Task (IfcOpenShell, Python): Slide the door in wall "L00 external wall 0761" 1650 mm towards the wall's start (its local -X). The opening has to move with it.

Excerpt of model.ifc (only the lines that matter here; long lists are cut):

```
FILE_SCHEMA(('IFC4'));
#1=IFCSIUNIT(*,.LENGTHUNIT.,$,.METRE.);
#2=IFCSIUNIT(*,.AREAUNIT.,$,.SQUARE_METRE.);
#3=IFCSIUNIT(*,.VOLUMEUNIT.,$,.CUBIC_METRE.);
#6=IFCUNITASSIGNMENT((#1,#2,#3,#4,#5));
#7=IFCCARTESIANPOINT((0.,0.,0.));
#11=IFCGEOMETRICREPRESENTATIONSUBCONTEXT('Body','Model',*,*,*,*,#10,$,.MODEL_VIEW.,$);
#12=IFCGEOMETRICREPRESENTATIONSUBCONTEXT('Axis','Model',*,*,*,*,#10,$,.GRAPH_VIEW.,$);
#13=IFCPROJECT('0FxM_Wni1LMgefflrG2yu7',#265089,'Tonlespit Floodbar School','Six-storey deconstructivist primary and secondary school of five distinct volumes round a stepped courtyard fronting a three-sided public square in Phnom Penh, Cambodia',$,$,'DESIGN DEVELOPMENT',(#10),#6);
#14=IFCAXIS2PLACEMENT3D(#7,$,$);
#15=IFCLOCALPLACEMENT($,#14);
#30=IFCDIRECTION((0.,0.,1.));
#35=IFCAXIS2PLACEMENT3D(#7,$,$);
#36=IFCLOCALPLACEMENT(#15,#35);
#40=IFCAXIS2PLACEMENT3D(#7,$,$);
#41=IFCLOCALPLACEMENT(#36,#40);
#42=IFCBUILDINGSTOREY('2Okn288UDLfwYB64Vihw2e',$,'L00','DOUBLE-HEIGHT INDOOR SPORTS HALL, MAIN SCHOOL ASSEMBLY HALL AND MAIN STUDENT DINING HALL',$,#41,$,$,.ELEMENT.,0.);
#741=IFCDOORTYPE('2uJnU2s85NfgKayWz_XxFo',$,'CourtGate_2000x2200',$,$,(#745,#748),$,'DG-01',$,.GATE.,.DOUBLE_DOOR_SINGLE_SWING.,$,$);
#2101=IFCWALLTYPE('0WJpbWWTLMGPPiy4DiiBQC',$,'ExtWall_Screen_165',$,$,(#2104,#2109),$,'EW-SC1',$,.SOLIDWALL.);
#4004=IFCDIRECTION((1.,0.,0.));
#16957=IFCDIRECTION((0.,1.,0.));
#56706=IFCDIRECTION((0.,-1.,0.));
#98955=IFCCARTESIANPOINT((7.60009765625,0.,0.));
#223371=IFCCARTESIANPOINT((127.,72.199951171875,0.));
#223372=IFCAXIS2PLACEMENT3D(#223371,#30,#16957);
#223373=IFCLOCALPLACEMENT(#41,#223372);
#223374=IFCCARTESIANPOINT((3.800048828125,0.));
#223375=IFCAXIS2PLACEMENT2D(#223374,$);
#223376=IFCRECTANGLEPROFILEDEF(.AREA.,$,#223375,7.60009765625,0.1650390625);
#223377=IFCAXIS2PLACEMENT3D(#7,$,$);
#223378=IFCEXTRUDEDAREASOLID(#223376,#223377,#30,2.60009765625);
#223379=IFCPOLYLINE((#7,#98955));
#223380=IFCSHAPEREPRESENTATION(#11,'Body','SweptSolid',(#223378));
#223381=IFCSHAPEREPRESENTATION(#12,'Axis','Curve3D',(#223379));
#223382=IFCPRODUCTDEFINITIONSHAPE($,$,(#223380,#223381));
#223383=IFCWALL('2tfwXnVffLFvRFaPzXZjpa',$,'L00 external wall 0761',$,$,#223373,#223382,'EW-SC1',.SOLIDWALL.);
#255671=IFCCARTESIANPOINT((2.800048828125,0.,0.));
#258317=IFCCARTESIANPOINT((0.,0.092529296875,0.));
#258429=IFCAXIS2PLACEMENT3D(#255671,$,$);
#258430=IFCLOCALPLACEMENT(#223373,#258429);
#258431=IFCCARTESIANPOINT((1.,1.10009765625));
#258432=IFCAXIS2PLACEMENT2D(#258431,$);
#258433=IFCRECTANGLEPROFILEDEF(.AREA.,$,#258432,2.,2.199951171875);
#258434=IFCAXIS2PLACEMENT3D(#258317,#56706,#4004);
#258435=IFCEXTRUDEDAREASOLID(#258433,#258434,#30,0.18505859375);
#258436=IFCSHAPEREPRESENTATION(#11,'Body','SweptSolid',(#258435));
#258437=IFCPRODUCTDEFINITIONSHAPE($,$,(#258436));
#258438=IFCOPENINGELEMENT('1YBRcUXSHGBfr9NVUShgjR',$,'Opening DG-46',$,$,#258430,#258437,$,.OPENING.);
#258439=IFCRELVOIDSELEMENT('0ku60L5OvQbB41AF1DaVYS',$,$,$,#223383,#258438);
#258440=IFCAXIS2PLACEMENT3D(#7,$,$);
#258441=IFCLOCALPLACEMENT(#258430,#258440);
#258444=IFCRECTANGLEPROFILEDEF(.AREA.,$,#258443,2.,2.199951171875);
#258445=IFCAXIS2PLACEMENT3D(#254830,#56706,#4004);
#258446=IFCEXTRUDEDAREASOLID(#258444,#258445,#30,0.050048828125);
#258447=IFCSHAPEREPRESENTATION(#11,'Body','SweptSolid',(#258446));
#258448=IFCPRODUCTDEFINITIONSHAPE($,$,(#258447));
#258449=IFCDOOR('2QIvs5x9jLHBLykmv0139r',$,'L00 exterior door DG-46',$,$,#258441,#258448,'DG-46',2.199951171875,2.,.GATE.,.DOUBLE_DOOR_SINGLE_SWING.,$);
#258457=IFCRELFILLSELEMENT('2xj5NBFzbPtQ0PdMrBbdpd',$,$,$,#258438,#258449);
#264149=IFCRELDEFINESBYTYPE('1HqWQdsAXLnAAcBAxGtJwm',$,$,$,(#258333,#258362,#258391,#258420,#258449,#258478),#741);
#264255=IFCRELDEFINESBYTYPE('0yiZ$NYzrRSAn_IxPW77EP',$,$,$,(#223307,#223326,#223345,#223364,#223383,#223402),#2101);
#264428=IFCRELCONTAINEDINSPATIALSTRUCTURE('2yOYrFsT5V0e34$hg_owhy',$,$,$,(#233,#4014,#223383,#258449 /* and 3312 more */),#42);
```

```python
import ifcopenshell
import ifcopenshell.api.geometry
import ifcopenshell.util.placement

model = ifcopenshell.open("model.ifc")

door = model.by_guid("2QIvs5x9jLHBLykmv0139r")
opening = door.FillsVoids[0].RelatingOpeningElement
wall = opening.VoidsElements[0].RelatingBuildingElement

wall_matrix = ifcopenshell.util.placement.get_local_placement(wall.ObjectPlacement)
shift = wall_matrix[:3, 0] * -1.65
before = ifcopenshell.util.placement.get_local_placement(door.ObjectPlacement)[:3, 3].copy()

# The door is placed relative to its opening, so it follows when the opening moves.
matrix = ifcopenshell.util.placement.get_local_placement(opening.ObjectPlacement)
matrix[:3, 3] += shift
ifcopenshell.api.geometry.edit_object_placement(
    model, product=opening, matrix=matrix, is_si=False, should_transform_children=True
)

after = ifcopenshell.util.placement.get_local_placement(door.ObjectPlacement)[:3, 3]
print("door moved by", (after - before).round(3) + 0.0)

model.write("model_rev.ifc")
```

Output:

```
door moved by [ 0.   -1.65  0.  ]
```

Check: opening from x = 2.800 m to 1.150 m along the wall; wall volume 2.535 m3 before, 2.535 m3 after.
